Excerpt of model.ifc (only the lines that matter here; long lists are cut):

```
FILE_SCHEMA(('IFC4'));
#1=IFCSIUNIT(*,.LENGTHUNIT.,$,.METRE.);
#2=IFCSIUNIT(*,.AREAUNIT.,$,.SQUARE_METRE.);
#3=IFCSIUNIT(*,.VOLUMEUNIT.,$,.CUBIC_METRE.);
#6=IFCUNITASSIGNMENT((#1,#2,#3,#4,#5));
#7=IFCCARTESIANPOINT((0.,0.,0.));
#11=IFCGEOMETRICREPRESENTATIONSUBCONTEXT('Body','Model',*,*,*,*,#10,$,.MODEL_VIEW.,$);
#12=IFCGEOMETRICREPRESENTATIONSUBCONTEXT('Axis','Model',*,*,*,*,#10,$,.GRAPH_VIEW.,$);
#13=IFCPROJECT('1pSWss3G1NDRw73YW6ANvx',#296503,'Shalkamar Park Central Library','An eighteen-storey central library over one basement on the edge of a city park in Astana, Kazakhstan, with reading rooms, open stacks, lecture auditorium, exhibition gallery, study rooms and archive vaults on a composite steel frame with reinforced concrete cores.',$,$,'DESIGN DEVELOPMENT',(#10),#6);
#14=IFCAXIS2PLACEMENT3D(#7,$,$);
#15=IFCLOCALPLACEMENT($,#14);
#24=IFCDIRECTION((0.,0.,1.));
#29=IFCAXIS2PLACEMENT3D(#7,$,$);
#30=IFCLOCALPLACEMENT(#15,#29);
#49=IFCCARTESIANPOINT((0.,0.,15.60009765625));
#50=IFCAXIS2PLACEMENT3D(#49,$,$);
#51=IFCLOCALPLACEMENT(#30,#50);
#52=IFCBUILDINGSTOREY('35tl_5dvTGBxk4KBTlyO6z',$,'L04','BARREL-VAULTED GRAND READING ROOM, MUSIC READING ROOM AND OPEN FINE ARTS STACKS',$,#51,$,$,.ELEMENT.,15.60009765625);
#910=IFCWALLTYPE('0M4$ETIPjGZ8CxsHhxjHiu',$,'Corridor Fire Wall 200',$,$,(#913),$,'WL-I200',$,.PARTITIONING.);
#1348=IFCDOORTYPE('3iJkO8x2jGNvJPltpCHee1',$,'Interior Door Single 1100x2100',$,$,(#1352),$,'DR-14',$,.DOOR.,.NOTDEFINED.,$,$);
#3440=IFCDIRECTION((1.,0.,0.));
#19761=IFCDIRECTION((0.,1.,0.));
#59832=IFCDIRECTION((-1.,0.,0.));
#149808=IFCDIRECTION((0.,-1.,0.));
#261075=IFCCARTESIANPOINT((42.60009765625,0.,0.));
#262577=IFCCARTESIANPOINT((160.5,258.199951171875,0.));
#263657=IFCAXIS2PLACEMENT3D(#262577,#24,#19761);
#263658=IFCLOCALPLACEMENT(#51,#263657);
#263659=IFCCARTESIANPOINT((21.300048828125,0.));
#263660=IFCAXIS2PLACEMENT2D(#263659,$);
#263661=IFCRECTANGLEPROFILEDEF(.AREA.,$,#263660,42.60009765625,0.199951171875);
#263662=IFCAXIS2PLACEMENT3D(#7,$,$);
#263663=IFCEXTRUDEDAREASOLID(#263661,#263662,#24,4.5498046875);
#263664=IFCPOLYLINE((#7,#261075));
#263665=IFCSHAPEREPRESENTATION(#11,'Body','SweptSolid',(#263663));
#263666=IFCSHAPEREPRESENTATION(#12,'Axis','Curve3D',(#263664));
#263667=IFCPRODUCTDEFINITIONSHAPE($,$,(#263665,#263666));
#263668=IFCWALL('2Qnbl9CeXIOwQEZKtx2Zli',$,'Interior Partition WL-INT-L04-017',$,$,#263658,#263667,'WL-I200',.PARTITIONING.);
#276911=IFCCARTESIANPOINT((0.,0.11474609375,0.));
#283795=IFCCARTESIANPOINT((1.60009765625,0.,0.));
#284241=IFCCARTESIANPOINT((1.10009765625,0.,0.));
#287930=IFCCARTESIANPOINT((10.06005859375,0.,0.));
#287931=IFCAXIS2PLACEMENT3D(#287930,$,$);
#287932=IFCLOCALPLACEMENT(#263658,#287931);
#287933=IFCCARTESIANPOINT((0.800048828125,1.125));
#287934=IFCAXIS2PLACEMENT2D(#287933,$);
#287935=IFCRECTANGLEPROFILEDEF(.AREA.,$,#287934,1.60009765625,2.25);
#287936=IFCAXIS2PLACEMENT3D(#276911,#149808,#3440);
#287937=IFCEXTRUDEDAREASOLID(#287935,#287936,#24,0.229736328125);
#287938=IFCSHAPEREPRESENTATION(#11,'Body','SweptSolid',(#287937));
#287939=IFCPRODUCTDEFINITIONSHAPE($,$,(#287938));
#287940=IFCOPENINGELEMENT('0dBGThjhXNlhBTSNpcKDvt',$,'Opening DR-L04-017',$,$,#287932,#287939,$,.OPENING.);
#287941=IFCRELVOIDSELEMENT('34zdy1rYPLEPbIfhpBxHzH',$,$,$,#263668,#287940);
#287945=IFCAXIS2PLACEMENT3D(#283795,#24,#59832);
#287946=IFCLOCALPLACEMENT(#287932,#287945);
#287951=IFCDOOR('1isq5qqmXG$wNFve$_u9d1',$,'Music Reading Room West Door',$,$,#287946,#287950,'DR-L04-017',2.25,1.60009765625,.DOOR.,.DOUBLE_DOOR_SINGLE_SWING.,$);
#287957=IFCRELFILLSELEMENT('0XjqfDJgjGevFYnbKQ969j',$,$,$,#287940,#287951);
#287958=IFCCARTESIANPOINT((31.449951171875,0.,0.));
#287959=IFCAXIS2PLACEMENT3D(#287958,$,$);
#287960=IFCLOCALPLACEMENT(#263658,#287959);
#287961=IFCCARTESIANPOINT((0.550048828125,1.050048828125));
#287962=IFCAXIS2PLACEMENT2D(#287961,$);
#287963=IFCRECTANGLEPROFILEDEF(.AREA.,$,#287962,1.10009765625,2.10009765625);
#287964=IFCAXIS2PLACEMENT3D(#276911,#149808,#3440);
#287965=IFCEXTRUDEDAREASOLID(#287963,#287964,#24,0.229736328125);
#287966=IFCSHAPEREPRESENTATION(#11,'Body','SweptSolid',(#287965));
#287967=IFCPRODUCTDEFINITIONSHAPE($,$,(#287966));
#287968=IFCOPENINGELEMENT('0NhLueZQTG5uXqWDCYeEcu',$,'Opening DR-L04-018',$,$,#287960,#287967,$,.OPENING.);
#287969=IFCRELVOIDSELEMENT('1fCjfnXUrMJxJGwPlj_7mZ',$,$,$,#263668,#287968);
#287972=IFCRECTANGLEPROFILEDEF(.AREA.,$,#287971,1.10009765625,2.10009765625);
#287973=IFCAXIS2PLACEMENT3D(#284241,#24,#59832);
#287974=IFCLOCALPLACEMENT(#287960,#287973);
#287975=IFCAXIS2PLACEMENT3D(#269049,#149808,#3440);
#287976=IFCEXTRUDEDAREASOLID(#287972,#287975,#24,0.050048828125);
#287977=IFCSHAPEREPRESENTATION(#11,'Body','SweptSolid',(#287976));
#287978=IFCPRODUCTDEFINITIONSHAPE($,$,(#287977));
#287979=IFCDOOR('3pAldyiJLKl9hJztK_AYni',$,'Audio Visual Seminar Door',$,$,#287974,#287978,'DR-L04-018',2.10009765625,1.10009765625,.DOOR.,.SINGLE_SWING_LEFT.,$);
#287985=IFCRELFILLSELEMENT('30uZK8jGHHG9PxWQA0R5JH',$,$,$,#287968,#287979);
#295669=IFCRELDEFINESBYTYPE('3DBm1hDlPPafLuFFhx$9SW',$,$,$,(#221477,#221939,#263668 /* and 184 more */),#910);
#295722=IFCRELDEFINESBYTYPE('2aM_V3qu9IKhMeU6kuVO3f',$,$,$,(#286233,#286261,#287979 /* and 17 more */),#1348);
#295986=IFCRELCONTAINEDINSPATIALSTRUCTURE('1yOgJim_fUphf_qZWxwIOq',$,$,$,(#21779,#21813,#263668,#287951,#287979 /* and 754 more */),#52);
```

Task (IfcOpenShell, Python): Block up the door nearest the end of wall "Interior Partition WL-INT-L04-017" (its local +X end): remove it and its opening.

```python
import ifcopenshell
import ifcopenshell.api.feature
import ifcopenshell.api.root
import ifcopenshell.geom
import ifcopenshell.util.shape

model = ifcopenshell.open("model.ifc")
settings = ifcopenshell.geom.settings()


def volume(element):
    """Net volume in cubic metres, openings subtracted."""
    shape = ifcopenshell.geom.create_shape(settings, element)
    return ifcopenshell.util.shape.get_volume(shape.geometry)


door = model.by_guid("3pAldyiJLKl9hJztK_AYni")
opening = door.FillsVoids[0].RelatingOpeningElement
wall = opening.VoidsElements[0].RelatingBuildingElement
before = volume(wall)

ifcopenshell.api.root.remove_product(model, product=door)
ifcopenshell.api.feature.remove_feature(model, feature=opening)

after = volume(wall)

print(f"wall volume {before:.3f} -> {after:.3f} m3")

model.write("model-out.ifc")
```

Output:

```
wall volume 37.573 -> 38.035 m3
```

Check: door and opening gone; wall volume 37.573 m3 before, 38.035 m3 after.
